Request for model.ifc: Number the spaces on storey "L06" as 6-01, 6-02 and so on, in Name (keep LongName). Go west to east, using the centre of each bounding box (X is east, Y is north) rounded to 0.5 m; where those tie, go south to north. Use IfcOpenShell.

First a look at what the model holds.

```python
import ifcopenshell
import ifcopenshell.util.element
import ifcopenshell.util.placement

model = ifcopenshell.open("model.ifc")
print(model.schema)
storey = next(s for s in model.by_type("IfcBuildingStorey") if s.Name == "L06")
spaces = [e for e in ifcopenshell.util.element.get_decomposition(storey) if e.is_a("IfcSpace")]
for e in sorted(spaces, key=lambda e: e.id()):
    origin = ifcopenshell.util.placement.get_local_placement(e.ObjectPlacement)[:3, 3]
    print(e.id(), e.Name, e.LongName, origin.round(2) + 0.0, sep=" | ")
```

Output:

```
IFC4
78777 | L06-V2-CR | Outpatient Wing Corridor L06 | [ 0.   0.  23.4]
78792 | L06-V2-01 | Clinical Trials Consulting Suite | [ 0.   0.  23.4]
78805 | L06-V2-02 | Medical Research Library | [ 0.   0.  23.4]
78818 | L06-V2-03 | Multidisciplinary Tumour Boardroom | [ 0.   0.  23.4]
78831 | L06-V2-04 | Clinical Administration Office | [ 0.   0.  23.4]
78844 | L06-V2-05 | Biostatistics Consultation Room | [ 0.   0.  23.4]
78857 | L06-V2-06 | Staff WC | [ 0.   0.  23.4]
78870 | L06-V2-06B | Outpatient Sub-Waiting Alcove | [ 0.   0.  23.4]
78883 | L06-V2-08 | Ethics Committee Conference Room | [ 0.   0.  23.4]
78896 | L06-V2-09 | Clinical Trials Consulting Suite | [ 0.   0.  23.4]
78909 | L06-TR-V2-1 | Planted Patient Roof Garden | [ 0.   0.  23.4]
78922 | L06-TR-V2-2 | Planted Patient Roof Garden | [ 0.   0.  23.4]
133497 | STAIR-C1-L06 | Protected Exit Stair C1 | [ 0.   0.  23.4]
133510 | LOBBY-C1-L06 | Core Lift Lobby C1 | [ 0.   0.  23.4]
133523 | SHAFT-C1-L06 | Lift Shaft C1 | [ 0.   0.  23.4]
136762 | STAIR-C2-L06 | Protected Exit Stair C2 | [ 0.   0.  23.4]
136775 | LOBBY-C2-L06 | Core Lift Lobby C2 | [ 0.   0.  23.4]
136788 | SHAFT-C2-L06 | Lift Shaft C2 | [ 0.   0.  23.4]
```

```python
import ifcopenshell
import ifcopenshell.geom
import ifcopenshell.util.element
import ifcopenshell.util.shape

model = ifcopenshell.open("model.ifc")
settings = ifcopenshell.geom.settings()
settings.set("use-world-coords", True)


def centre(element):
    shape = ifcopenshell.geom.create_shape(settings, element)
    return ifcopenshell.util.shape.get_bbox_centroid(shape.geometry)


storey = next(s for s in model.by_type("IfcBuildingStorey") if s.Name == "L06")
spaces = [e for e in ifcopenshell.util.element.get_decomposition(storey) if e.is_a("IfcSpace")]

# Insertion points can sit at a corner or the storey origin, so sort by the geometry (in metres).
centres = {e: centre(e) for e in spaces}
spaces.sort(key=lambda e: (round(centres[e][0] / 0.5), centres[e][1]))

for i, e in enumerate(spaces, start=1):
    number = f"6-{i:02d}"
    e.Name = number
    print(e.id(), number)

model.write("model_v2.ifc")
```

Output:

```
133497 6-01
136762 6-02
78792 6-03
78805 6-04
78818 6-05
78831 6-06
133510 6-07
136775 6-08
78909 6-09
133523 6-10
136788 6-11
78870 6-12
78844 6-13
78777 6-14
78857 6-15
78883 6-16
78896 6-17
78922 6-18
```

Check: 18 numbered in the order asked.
